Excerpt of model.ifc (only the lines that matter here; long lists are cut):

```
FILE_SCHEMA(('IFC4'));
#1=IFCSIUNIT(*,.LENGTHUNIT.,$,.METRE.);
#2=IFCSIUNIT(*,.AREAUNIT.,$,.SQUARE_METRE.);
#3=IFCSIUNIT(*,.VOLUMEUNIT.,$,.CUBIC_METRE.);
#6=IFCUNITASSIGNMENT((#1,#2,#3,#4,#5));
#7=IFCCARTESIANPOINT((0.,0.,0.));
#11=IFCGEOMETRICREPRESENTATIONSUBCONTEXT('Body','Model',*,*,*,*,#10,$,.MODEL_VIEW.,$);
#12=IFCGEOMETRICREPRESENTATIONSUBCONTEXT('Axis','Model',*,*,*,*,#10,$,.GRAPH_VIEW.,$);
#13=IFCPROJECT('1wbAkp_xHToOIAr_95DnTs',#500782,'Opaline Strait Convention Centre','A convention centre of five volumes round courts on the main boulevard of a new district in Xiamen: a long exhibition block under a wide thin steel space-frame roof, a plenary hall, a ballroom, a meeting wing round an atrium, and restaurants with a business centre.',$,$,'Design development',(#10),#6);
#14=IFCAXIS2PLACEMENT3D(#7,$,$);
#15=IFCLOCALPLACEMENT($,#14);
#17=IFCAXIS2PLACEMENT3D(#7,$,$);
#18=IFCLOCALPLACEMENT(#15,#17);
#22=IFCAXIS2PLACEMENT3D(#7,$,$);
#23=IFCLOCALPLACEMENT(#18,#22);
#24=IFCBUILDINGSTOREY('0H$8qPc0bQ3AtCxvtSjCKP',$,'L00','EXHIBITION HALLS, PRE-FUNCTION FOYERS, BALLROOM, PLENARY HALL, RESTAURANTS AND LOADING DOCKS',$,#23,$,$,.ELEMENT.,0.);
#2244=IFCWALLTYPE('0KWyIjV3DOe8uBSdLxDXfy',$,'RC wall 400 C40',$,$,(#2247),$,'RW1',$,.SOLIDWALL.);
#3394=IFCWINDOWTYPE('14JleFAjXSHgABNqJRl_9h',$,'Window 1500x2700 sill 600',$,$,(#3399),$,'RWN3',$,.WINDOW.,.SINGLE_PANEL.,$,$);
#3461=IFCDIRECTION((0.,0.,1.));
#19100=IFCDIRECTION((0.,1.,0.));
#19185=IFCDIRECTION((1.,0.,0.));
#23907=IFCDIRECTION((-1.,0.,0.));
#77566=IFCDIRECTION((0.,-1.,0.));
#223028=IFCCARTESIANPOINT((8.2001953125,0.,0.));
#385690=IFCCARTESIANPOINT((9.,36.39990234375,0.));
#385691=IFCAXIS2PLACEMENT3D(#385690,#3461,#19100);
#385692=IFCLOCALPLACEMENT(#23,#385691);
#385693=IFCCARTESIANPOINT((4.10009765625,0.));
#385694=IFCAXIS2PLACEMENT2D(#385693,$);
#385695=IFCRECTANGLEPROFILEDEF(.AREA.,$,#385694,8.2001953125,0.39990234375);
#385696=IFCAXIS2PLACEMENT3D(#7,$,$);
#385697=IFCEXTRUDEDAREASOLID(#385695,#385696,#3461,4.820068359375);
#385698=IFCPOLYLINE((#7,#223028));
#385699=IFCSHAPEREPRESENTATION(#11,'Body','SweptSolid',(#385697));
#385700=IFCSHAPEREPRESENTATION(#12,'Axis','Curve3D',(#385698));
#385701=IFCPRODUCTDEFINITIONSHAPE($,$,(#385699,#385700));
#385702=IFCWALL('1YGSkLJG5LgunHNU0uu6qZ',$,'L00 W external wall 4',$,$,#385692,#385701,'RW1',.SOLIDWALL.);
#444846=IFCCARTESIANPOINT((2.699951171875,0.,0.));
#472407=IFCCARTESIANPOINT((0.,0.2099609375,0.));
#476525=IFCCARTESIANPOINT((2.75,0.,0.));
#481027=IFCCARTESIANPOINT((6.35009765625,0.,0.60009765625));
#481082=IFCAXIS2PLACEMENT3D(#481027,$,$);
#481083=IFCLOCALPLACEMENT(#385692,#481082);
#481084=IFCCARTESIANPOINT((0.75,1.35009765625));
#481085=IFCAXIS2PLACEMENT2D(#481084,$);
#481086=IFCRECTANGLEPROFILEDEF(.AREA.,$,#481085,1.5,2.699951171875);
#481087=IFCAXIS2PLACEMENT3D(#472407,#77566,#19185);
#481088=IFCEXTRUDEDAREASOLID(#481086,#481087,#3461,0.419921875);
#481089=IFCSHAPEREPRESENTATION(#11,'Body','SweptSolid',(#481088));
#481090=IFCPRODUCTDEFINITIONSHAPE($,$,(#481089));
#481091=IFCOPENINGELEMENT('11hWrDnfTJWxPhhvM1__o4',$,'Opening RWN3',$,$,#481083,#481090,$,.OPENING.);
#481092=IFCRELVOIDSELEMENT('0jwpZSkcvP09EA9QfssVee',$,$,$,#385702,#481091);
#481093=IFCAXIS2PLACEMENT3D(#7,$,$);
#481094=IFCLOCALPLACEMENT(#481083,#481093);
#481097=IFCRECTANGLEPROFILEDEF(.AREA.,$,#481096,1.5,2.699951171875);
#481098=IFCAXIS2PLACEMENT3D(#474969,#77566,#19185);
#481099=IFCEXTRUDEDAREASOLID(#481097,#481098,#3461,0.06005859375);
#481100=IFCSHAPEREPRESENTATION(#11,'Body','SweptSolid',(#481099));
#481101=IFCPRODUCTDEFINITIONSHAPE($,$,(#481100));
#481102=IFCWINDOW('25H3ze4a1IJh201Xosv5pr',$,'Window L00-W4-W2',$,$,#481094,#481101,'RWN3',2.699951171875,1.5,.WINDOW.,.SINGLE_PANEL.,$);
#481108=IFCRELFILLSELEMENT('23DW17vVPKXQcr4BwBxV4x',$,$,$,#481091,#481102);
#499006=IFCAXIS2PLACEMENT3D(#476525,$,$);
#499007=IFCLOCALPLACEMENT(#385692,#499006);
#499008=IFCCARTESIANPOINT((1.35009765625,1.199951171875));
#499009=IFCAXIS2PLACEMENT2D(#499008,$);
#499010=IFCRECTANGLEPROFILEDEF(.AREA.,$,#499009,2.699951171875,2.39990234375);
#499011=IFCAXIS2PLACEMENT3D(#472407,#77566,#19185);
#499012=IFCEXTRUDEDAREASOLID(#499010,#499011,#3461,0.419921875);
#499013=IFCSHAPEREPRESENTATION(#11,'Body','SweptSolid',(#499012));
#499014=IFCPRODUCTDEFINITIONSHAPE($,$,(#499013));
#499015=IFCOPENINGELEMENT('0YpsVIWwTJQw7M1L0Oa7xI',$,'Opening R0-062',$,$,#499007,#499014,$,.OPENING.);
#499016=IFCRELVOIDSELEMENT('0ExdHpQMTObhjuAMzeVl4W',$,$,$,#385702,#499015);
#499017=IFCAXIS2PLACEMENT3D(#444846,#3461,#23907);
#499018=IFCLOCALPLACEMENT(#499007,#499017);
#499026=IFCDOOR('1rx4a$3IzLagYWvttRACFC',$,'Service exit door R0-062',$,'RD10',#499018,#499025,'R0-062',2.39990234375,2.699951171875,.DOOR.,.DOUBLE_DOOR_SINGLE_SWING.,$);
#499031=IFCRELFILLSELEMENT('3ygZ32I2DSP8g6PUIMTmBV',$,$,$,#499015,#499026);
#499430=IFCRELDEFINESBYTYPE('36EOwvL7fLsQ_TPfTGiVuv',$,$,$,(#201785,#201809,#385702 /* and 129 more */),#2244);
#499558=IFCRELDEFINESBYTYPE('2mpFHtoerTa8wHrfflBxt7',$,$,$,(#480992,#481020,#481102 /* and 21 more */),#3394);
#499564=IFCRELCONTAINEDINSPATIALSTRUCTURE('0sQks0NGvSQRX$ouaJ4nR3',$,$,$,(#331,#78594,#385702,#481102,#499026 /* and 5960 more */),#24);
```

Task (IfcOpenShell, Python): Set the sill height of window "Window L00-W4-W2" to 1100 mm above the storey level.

```python
import numpy as np
import ifcopenshell
import ifcopenshell.api.geometry
import ifcopenshell.geom
import ifcopenshell.util.element
import ifcopenshell.util.placement
import ifcopenshell.util.shape
import ifcopenshell.util.unit

model = ifcopenshell.open("model.ifc")
unit_scale = ifcopenshell.util.unit.calculate_unit_scale(model)

window = model.by_guid("25H3ze4a1IJh201Xosv5pr")
opening = window.FillsVoids[0].RelatingOpeningElement
storey = ifcopenshell.util.element.get_container(window, ifc_class="IfcBuildingStorey")
level = ifcopenshell.util.placement.get_local_placement(storey.ObjectPlacement)[2, 3]

# The opening's origin need not be at the sill, so measure its lowest point.
shape = ifcopenshell.geom.create_shape(ifcopenshell.geom.settings(), opening)
bottom = ifcopenshell.util.shape.get_shape_bottom_elevation(shape, shape.geometry) / unit_scale
dz = level + 1.1 - bottom

shift = np.array([0.0, 0.0, dz])
# The window is placed relative to its opening, so it follows when the opening moves.
matrix = ifcopenshell.util.placement.get_local_placement(opening.ObjectPlacement)
matrix[:3, 3] += shift
ifcopenshell.api.geometry.edit_object_placement(
    model, product=opening, matrix=matrix, is_si=False, should_transform_children=True
)

print(f"moved by {dz * unit_scale:+.3f} m")

model.write("model_edited.ifc")
```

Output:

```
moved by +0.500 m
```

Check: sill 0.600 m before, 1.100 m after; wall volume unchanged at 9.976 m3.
